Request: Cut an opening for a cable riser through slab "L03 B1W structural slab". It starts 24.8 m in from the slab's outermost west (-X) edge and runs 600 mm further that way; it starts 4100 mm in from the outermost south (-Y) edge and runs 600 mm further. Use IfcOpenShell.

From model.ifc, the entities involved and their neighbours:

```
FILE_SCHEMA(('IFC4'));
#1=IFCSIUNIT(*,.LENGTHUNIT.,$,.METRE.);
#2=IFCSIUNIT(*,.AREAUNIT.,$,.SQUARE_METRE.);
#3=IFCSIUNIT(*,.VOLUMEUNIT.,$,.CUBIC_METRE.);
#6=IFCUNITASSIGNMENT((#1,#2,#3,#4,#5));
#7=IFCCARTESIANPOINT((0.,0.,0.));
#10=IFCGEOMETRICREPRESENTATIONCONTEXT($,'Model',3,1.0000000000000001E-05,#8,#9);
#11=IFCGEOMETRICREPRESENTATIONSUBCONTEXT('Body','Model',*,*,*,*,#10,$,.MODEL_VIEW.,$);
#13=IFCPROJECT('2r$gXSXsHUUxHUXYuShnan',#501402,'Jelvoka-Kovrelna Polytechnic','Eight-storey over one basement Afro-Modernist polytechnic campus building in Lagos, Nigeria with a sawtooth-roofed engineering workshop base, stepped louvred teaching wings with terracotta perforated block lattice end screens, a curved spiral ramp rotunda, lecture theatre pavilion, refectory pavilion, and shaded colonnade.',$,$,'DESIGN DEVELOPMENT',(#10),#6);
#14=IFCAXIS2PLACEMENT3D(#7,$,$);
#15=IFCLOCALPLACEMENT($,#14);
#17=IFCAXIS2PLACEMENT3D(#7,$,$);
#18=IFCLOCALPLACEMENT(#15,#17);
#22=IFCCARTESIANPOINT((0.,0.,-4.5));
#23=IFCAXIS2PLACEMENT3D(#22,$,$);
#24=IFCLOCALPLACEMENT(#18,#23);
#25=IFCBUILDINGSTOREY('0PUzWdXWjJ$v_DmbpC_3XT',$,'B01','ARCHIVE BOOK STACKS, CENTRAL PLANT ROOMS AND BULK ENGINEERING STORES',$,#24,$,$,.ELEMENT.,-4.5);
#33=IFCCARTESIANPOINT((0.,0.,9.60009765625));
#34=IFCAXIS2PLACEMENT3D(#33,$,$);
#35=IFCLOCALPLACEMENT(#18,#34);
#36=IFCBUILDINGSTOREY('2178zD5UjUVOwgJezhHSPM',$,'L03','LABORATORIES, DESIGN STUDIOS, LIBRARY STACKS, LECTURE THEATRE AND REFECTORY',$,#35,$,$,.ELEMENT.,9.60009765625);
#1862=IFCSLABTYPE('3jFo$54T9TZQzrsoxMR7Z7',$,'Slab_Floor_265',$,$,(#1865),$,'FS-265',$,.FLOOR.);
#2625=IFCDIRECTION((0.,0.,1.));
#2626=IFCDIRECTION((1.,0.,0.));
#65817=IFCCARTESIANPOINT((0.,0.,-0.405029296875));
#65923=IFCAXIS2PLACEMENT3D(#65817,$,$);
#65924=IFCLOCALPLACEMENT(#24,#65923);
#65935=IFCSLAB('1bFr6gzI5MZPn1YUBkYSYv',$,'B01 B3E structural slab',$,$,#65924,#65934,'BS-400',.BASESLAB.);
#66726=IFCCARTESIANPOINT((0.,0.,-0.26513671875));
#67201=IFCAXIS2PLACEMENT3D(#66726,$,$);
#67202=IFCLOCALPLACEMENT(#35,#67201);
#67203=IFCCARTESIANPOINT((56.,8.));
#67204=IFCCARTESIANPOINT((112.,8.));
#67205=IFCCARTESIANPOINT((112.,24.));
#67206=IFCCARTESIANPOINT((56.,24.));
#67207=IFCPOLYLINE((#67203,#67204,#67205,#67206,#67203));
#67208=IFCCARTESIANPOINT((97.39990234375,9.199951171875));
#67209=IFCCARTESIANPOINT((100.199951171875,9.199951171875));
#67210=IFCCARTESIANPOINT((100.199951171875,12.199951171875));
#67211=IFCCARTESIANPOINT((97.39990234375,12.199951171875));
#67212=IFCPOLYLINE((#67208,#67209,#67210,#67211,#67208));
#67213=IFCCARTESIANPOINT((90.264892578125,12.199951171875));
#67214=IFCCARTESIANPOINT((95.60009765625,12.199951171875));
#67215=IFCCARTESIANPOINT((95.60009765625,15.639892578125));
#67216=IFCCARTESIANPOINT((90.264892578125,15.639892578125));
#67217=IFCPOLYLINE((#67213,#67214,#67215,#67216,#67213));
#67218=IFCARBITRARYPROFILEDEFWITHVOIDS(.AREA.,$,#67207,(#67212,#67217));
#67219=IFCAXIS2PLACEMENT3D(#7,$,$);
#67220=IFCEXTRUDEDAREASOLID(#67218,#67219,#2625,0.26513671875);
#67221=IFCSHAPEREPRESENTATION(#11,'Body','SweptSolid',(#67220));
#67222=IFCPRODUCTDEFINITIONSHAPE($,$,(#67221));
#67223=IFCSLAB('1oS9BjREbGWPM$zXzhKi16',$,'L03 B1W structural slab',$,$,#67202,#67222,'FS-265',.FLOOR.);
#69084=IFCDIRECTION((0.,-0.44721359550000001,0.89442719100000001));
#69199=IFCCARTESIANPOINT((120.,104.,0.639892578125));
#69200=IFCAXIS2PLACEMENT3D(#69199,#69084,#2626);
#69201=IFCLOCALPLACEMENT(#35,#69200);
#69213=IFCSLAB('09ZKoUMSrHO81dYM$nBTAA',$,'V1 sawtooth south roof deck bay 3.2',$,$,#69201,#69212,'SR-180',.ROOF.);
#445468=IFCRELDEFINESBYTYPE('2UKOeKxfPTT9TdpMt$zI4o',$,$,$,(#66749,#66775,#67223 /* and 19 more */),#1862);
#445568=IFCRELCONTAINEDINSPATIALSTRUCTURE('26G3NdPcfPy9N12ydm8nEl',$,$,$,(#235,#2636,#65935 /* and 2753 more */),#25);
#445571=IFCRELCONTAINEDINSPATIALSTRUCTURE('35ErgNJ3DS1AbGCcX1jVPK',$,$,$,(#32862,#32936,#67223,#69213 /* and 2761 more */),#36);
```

```python
import numpy as np
import ifcopenshell
import ifcopenshell.api.feature
import ifcopenshell.api.geometry
import ifcopenshell.api.root
import ifcopenshell.geom
import ifcopenshell.util.placement
import ifcopenshell.util.representation
import ifcopenshell.util.shape
import ifcopenshell.util.unit

model = ifcopenshell.open("model.ifc")
unit_scale = ifcopenshell.util.unit.calculate_unit_scale(model)
settings = ifcopenshell.geom.settings()


def volume(element):
    """Net volume in cubic metres, openings subtracted."""
    shape = ifcopenshell.geom.create_shape(settings, element)
    return ifcopenshell.util.shape.get_volume(shape.geometry)


slab = model.by_guid("1oS9BjREbGWPM$zXzhKi16")
before = volume(slab)

# Extent in the slab's own axes, in metres. The edges named are its -X and -Y sides.
slab_shape = ifcopenshell.geom.create_shape(settings, slab)
vertices = ifcopenshell.util.shape.get_vertices(slab_shape.geometry)
x_min, y_min, bottom = vertices.min(axis=0)
top = vertices[:, 2].max()

opening = ifcopenshell.api.root.create_entity(model, ifc_class="IfcOpeningElement", name="Cable riser opening", predefined_type="OPENING")
context = ifcopenshell.util.representation.get_context(model, "Model", "Body", "MODEL_VIEW")
width, depth = 0.6, 0.6
outline = [(0.0, 0.0), (width, 0.0), (width, depth), (0.0, depth), (0.0, 0.0)]
# Overshoot both faces by 50 mm so the cut is clean.
shape = ifcopenshell.api.geometry.add_slab_representation(
    model, context=context, depth=top - bottom + 0.1, polyline=outline
)
ifcopenshell.api.geometry.assign_representation(model, product=opening, representation=shape)

matrix = ifcopenshell.util.placement.get_local_placement(slab.ObjectPlacement)
matrix[:, 3] = matrix @ np.append(np.array([x_min + 24.8, y_min + 4.1, bottom - 0.05]) / unit_scale, 1.0)
ifcopenshell.api.geometry.edit_object_placement(model, product=opening, matrix=matrix, is_si=False)
ifcopenshell.api.feature.add_feature(model, feature=opening, element=slab)

after = volume(slab)

print(f"slab volume {before:.3f} -> {after:.3f} m3")

model.write("model_updated.ifc")
```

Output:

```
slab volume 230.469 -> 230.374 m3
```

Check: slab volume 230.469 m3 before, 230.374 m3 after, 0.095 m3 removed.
